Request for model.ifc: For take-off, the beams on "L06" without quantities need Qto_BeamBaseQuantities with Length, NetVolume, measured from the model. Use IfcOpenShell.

First a look at what the model holds.

```python
import ifcopenshell
import ifcopenshell.util.element
import ifcopenshell.util.unit

model = ifcopenshell.open("model.ifc")
print(model.schema)
for unit_type in ("LENGTHUNIT", "AREAUNIT", "VOLUMEUNIT"):
    print(unit_type, ifcopenshell.util.unit.calculate_unit_scale(model, unit_type))
storey = next(s for s in model.by_type("IfcBuildingStorey") if s.Name == "L06")
beams = [e for e in ifcopenshell.util.element.get_decomposition(storey) if e.is_a("IfcBeam")]
for e in sorted(beams, key=lambda e: e.id()):
    print(e.id(), e.is_a(), e.Name, list(ifcopenshell.util.element.get_psets(e, qtos_only=True)), sep=" | ")
```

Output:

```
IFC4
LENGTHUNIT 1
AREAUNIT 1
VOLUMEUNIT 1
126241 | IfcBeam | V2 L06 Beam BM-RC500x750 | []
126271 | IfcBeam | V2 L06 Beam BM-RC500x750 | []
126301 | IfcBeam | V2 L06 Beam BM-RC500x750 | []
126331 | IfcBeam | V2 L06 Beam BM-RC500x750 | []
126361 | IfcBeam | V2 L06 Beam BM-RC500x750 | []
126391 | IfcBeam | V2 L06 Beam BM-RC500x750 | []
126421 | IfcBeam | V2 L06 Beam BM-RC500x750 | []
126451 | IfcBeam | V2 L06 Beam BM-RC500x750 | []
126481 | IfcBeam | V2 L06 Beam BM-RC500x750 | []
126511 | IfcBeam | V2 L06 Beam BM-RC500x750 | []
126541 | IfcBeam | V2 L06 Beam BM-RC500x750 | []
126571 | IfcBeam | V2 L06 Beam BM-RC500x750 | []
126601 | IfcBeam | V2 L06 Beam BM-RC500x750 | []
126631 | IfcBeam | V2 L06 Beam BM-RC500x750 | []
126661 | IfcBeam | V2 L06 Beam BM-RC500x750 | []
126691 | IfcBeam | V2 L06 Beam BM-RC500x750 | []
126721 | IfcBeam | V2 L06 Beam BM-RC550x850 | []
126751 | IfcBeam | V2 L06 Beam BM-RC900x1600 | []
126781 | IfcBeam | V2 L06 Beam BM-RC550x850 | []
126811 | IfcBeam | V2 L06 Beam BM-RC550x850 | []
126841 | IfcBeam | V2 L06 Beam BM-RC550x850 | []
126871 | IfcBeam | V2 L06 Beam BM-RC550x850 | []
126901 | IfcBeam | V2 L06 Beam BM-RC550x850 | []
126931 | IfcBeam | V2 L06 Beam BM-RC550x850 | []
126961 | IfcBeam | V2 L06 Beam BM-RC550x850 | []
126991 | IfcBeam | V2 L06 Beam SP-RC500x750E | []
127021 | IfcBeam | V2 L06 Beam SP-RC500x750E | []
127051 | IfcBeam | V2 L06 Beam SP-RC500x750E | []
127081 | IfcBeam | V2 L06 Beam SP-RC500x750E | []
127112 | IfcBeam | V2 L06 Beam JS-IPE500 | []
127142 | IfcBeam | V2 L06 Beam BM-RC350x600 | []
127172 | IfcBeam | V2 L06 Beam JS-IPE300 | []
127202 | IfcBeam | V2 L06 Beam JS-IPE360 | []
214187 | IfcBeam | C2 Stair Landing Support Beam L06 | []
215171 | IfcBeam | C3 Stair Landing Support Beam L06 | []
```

```python
import ifcopenshell
import ifcopenshell.api.pset
import ifcopenshell.geom
import ifcopenshell.util.element
import ifcopenshell.util.shape
import ifcopenshell.util.unit

model = ifcopenshell.open("model.ifc")
unit_scale = ifcopenshell.util.unit.calculate_unit_scale(model)
volume_scale = ifcopenshell.util.unit.calculate_unit_scale(model, "VOLUMEUNIT")
settings = ifcopenshell.geom.settings()

storey = next(s for s in model.by_type("IfcBuildingStorey") if s.Name == "L06")
beams = [e for e in ifcopenshell.util.element.get_decomposition(storey) if e.is_a("IfcBeam")]

for e in sorted(beams, key=lambda e: e.id()):
    if ifcopenshell.util.element.get_psets(e, qtos_only=True, should_inherit=False):
        continue
    # Geometry comes back in metres, in the element's own axes.
    shape = ifcopenshell.geom.create_shape(settings, e)
    values = {
        "Length": ifcopenshell.util.shape.get_max_xyz(shape.geometry) / unit_scale,
        "NetVolume": ifcopenshell.util.shape.get_volume(shape.geometry) / volume_scale,
    }
    qto = ifcopenshell.api.pset.add_qto(model, product=e, name="Qto_BeamBaseQuantities")
    ifcopenshell.api.pset.edit_qto(model, qto=qto, properties=values)
    print(e.id(), {k: round(v, 3) for k, v in values.items()})

model.write("model-out.ifc")
```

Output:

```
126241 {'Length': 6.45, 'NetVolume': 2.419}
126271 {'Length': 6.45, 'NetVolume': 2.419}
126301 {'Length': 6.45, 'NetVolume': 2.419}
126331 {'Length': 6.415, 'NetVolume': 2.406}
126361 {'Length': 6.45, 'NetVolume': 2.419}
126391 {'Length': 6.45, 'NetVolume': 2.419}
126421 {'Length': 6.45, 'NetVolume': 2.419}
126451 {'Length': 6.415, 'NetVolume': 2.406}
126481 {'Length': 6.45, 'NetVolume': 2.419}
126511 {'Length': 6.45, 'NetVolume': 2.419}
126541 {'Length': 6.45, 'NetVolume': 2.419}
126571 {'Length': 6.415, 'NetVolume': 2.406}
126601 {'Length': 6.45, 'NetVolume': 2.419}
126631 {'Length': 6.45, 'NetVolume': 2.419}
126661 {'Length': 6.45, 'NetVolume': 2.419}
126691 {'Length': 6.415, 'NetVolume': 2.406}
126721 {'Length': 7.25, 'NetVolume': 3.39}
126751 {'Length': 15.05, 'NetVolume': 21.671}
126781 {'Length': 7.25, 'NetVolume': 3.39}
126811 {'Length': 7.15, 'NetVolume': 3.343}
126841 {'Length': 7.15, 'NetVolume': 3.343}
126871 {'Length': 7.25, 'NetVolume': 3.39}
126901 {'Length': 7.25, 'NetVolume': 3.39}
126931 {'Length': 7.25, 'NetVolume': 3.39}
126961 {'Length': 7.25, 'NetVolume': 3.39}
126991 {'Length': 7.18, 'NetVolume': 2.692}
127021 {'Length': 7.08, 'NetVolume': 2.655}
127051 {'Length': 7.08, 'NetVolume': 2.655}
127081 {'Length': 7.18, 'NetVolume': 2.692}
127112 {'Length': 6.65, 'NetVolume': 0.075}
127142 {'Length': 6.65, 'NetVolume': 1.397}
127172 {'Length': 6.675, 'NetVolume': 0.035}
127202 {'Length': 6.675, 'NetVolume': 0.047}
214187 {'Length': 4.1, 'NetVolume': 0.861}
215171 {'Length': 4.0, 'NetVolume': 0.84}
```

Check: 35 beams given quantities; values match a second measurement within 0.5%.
